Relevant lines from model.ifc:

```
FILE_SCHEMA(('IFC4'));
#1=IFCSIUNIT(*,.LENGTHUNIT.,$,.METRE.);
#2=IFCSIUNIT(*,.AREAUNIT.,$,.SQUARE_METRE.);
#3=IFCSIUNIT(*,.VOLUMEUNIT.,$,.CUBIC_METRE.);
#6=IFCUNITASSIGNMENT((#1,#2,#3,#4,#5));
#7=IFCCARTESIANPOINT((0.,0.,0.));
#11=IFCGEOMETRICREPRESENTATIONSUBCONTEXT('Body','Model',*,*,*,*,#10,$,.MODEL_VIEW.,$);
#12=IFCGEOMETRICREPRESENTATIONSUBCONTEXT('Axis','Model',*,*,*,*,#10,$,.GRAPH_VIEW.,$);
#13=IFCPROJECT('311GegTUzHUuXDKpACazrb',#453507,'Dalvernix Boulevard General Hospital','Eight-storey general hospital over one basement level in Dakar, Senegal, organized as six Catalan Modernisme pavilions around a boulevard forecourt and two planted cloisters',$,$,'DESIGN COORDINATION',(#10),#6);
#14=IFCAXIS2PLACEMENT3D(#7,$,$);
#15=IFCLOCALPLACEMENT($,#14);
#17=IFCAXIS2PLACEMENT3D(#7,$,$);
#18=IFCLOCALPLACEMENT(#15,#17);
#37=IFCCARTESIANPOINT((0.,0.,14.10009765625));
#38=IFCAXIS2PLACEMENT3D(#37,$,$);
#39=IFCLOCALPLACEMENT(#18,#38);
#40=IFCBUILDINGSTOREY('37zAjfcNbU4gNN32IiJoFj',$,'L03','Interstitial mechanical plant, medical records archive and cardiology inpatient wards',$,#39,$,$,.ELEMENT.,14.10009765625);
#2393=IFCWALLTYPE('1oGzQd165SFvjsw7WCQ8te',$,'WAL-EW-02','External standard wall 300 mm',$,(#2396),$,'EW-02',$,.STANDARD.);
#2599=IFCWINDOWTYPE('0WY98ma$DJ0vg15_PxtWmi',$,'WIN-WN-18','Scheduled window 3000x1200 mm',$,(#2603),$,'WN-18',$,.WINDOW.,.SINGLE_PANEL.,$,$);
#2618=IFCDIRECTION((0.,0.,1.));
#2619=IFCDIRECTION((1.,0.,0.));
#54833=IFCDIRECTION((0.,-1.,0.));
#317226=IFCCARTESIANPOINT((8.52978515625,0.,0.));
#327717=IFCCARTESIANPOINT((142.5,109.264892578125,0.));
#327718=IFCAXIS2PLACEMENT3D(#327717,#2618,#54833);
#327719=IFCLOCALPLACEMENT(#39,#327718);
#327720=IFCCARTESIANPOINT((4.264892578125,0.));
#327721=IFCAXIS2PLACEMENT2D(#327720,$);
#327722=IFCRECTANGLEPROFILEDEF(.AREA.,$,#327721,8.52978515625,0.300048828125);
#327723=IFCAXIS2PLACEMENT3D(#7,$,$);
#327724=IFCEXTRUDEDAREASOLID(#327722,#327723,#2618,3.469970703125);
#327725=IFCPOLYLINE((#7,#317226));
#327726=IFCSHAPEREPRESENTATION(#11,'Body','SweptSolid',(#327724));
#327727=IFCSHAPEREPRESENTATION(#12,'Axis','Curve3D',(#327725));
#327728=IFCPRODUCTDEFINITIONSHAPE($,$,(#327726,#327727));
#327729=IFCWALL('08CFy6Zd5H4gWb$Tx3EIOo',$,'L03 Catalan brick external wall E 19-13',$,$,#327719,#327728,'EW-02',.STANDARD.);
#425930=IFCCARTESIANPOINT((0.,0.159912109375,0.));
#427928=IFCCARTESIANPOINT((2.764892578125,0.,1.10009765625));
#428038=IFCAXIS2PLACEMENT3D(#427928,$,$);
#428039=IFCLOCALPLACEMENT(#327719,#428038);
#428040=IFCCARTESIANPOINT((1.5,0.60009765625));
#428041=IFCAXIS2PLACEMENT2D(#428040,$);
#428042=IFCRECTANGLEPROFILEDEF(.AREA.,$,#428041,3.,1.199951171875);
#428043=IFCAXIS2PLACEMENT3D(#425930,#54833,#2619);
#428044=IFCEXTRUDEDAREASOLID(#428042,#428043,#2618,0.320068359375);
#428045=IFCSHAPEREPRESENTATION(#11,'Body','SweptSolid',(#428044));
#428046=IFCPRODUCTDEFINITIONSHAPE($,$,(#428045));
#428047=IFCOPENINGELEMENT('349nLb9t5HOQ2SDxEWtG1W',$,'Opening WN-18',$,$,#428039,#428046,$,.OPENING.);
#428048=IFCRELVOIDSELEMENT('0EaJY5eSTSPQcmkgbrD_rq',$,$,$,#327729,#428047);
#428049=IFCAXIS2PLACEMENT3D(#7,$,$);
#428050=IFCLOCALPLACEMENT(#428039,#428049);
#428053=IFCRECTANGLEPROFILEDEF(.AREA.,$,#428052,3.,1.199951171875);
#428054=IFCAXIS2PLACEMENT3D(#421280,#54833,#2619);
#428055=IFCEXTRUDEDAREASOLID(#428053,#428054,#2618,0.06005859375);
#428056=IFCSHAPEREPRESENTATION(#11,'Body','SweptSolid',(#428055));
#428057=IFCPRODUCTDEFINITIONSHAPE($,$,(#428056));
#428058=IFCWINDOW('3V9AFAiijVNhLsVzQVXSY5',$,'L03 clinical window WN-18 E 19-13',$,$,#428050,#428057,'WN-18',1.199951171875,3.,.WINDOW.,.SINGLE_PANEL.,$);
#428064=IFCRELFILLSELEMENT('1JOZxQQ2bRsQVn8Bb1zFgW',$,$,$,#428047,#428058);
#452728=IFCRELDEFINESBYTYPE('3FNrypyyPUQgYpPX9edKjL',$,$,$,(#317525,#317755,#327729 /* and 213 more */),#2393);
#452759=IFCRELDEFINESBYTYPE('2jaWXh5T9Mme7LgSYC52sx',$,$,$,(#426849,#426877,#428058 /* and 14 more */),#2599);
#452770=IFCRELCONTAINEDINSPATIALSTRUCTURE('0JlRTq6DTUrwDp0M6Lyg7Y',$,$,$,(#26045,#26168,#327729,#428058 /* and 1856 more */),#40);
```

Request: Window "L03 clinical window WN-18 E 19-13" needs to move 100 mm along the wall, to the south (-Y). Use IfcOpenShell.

```python
import ifcopenshell
import ifcopenshell.api.geometry
import ifcopenshell.util.placement
import ifcopenshell.util.unit

model = ifcopenshell.open("model.ifc")
unit_scale = ifcopenshell.util.unit.calculate_unit_scale(model)

window = model.by_guid("3V9AFAiijVNhLsVzQVXSY5")
opening = window.FillsVoids[0].RelatingOpeningElement
wall = opening.VoidsElements[0].RelatingBuildingElement

wall_matrix = ifcopenshell.util.placement.get_local_placement(wall.ObjectPlacement)
shift = wall_matrix[:3, 0] * 0.1 / unit_scale
before = ifcopenshell.util.placement.get_local_placement(window.ObjectPlacement)[:3, 3].copy()

# The window is placed relative to its opening, so it follows when the opening moves.
matrix = ifcopenshell.util.placement.get_local_placement(opening.ObjectPlacement)
matrix[:3, 3] += shift
ifcopenshell.api.geometry.edit_object_placement(
    model, product=opening, matrix=matrix, is_si=False, should_transform_children=True
)

after = ifcopenshell.util.placement.get_local_placement(window.ObjectPlacement)[:3, 3]
print("window moved by", (after - before).round(3) + 0.0)

model.write("model_updated.ifc")
```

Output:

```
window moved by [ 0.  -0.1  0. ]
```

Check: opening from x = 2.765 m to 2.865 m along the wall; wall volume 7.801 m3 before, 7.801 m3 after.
